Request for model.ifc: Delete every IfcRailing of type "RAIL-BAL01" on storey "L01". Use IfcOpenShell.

First a look at what the model holds.

```python
import ifcopenshell
import ifcopenshell.util.element

model = ifcopenshell.open("model.ifc")
print(model.schema)
storey = next(s for s in model.by_type("IfcBuildingStorey") if s.Name == "L01")
railings = [e for e in ifcopenshell.util.element.get_decomposition(storey) if e.is_a("IfcRailing")]
seen = {}
for e in railings:
    element_type = ifcopenshell.util.element.get_type(e)
    name = element_type.Name if element_type not in (None, e) else None
    seen[name] = seen.get(name, 0) + 1
for name, count in sorted(seen.items(), key=str):
    print(count, "x", name)
```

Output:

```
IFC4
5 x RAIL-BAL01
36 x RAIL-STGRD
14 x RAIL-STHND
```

```python
import ifcopenshell
import ifcopenshell.api.root
import ifcopenshell.util.element

model = ifcopenshell.open("model.ifc")

storey = next(s for s in model.by_type("IfcBuildingStorey") if s.Name == "L01")
railings = [e for e in ifcopenshell.util.element.get_decomposition(storey) if e.is_a("IfcRailing")]
targets = [e for e in railings if (t := ifcopenshell.util.element.get_type(e)) not in (None, e) and t.Name == "RAIL-BAL01"]

for e in targets:
    ifcopenshell.api.root.remove_product(model, product=e)
print(len(targets), "removed")

model.write("model_v2.ifc")
```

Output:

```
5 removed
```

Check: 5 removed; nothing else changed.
